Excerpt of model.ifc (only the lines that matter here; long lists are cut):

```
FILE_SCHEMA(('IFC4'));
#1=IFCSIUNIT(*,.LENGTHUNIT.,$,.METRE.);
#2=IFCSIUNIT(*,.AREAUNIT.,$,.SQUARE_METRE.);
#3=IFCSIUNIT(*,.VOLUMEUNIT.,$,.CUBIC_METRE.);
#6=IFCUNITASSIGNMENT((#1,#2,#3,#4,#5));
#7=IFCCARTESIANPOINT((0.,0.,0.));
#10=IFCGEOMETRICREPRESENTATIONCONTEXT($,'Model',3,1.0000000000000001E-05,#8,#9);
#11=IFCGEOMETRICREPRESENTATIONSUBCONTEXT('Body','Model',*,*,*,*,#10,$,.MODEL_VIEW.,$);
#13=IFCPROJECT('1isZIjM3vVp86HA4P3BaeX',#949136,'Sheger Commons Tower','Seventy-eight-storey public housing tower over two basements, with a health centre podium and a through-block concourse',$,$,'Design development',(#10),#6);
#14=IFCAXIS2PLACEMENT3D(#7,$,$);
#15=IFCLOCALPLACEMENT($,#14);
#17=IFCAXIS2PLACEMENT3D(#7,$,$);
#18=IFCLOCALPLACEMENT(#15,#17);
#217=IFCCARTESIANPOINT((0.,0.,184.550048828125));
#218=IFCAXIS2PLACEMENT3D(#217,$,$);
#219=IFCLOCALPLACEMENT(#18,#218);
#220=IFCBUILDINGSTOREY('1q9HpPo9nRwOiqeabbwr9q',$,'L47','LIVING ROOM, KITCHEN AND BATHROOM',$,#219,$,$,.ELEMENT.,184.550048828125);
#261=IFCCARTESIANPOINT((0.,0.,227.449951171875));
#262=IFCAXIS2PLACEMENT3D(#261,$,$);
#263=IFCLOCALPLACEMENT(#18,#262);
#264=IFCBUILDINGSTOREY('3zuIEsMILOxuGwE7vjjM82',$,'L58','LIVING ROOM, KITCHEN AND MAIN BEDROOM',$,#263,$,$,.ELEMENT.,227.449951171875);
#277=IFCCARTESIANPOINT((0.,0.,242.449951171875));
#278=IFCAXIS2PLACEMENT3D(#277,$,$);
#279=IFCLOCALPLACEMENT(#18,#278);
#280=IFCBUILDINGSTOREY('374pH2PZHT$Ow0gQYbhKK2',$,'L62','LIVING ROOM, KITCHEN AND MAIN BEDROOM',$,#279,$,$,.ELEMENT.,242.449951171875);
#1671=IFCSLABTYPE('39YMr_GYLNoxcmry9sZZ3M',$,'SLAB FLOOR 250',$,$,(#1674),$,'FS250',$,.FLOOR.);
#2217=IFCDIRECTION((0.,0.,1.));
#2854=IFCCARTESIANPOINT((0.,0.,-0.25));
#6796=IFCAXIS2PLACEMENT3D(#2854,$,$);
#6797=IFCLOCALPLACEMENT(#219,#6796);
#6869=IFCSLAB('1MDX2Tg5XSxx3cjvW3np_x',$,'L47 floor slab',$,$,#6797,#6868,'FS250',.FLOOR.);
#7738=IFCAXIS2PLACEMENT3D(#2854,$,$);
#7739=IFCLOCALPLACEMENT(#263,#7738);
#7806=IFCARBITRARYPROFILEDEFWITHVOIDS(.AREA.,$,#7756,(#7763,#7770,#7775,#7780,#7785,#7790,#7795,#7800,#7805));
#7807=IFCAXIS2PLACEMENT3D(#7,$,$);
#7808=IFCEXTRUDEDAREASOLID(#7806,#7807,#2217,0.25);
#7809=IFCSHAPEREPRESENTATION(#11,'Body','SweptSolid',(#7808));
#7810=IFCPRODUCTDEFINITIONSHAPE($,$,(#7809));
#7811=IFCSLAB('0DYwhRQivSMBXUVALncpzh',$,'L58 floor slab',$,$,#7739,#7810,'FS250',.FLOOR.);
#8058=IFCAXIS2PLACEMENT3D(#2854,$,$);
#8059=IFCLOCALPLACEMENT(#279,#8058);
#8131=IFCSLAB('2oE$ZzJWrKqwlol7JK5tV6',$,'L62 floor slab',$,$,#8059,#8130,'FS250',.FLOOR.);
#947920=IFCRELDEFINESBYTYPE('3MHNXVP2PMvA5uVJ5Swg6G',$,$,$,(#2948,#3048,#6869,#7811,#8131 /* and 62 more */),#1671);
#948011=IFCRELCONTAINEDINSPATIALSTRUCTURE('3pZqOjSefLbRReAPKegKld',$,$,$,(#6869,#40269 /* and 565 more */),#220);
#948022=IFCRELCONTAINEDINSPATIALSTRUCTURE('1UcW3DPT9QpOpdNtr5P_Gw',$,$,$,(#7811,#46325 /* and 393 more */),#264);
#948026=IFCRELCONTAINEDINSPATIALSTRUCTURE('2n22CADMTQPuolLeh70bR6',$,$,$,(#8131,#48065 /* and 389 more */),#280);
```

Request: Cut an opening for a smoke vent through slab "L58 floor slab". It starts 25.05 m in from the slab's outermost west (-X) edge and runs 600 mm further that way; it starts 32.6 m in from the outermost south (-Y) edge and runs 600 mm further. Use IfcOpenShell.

```python
import numpy as np
import ifcopenshell
import ifcopenshell.api.feature
import ifcopenshell.api.geometry
import ifcopenshell.api.root
import ifcopenshell.geom
import ifcopenshell.util.placement
import ifcopenshell.util.representation
import ifcopenshell.util.shape
import ifcopenshell.util.unit

model = ifcopenshell.open("model.ifc")
unit_scale = ifcopenshell.util.unit.calculate_unit_scale(model)
settings = ifcopenshell.geom.settings()


def volume(element):
    """Net volume in cubic metres, openings subtracted."""
    shape = ifcopenshell.geom.create_shape(settings, element)
    return ifcopenshell.util.shape.get_volume(shape.geometry)


slab = model.by_id(7811)
before = volume(slab)

# Extent in the slab's own axes, in metres. The edges named are its -X and -Y sides.
slab_shape = ifcopenshell.geom.create_shape(settings, slab)
vertices = ifcopenshell.util.shape.get_vertices(slab_shape.geometry)
x_min, y_min, bottom = vertices.min(axis=0)
top = vertices[:, 2].max()

opening = ifcopenshell.api.root.create_entity(model, ifc_class="IfcOpeningElement", name="Smoke vent opening", predefined_type="OPENING")
context = ifcopenshell.util.representation.get_context(model, "Model", "Body", "MODEL_VIEW")
width, depth = 0.6, 0.6
outline = [(0.0, 0.0), (width, 0.0), (width, depth), (0.0, depth), (0.0, 0.0)]
# Overshoot both faces by 50 mm so the cut is clean.
shape = ifcopenshell.api.geometry.add_slab_representation(
    model, context=context, depth=top - bottom + 0.1, polyline=outline
)
ifcopenshell.api.geometry.assign_representation(model, product=opening, representation=shape)

matrix = ifcopenshell.util.placement.get_local_placement(slab.ObjectPlacement)
matrix[:, 3] = matrix @ np.append(np.array([x_min + 25.05, y_min + 32.6, bottom - 0.05]) / unit_scale, 1.0)
ifcopenshell.api.geometry.edit_object_placement(model, product=opening, matrix=matrix, is_si=False)
ifcopenshell.api.feature.add_feature(model, feature=opening, element=slab)

after = volume(slab)

print(f"slab volume {before:.3f} -> {after:.3f} m3")

model.write("model_rev.ifc")
```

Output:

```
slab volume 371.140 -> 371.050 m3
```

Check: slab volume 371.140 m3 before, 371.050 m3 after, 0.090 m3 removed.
